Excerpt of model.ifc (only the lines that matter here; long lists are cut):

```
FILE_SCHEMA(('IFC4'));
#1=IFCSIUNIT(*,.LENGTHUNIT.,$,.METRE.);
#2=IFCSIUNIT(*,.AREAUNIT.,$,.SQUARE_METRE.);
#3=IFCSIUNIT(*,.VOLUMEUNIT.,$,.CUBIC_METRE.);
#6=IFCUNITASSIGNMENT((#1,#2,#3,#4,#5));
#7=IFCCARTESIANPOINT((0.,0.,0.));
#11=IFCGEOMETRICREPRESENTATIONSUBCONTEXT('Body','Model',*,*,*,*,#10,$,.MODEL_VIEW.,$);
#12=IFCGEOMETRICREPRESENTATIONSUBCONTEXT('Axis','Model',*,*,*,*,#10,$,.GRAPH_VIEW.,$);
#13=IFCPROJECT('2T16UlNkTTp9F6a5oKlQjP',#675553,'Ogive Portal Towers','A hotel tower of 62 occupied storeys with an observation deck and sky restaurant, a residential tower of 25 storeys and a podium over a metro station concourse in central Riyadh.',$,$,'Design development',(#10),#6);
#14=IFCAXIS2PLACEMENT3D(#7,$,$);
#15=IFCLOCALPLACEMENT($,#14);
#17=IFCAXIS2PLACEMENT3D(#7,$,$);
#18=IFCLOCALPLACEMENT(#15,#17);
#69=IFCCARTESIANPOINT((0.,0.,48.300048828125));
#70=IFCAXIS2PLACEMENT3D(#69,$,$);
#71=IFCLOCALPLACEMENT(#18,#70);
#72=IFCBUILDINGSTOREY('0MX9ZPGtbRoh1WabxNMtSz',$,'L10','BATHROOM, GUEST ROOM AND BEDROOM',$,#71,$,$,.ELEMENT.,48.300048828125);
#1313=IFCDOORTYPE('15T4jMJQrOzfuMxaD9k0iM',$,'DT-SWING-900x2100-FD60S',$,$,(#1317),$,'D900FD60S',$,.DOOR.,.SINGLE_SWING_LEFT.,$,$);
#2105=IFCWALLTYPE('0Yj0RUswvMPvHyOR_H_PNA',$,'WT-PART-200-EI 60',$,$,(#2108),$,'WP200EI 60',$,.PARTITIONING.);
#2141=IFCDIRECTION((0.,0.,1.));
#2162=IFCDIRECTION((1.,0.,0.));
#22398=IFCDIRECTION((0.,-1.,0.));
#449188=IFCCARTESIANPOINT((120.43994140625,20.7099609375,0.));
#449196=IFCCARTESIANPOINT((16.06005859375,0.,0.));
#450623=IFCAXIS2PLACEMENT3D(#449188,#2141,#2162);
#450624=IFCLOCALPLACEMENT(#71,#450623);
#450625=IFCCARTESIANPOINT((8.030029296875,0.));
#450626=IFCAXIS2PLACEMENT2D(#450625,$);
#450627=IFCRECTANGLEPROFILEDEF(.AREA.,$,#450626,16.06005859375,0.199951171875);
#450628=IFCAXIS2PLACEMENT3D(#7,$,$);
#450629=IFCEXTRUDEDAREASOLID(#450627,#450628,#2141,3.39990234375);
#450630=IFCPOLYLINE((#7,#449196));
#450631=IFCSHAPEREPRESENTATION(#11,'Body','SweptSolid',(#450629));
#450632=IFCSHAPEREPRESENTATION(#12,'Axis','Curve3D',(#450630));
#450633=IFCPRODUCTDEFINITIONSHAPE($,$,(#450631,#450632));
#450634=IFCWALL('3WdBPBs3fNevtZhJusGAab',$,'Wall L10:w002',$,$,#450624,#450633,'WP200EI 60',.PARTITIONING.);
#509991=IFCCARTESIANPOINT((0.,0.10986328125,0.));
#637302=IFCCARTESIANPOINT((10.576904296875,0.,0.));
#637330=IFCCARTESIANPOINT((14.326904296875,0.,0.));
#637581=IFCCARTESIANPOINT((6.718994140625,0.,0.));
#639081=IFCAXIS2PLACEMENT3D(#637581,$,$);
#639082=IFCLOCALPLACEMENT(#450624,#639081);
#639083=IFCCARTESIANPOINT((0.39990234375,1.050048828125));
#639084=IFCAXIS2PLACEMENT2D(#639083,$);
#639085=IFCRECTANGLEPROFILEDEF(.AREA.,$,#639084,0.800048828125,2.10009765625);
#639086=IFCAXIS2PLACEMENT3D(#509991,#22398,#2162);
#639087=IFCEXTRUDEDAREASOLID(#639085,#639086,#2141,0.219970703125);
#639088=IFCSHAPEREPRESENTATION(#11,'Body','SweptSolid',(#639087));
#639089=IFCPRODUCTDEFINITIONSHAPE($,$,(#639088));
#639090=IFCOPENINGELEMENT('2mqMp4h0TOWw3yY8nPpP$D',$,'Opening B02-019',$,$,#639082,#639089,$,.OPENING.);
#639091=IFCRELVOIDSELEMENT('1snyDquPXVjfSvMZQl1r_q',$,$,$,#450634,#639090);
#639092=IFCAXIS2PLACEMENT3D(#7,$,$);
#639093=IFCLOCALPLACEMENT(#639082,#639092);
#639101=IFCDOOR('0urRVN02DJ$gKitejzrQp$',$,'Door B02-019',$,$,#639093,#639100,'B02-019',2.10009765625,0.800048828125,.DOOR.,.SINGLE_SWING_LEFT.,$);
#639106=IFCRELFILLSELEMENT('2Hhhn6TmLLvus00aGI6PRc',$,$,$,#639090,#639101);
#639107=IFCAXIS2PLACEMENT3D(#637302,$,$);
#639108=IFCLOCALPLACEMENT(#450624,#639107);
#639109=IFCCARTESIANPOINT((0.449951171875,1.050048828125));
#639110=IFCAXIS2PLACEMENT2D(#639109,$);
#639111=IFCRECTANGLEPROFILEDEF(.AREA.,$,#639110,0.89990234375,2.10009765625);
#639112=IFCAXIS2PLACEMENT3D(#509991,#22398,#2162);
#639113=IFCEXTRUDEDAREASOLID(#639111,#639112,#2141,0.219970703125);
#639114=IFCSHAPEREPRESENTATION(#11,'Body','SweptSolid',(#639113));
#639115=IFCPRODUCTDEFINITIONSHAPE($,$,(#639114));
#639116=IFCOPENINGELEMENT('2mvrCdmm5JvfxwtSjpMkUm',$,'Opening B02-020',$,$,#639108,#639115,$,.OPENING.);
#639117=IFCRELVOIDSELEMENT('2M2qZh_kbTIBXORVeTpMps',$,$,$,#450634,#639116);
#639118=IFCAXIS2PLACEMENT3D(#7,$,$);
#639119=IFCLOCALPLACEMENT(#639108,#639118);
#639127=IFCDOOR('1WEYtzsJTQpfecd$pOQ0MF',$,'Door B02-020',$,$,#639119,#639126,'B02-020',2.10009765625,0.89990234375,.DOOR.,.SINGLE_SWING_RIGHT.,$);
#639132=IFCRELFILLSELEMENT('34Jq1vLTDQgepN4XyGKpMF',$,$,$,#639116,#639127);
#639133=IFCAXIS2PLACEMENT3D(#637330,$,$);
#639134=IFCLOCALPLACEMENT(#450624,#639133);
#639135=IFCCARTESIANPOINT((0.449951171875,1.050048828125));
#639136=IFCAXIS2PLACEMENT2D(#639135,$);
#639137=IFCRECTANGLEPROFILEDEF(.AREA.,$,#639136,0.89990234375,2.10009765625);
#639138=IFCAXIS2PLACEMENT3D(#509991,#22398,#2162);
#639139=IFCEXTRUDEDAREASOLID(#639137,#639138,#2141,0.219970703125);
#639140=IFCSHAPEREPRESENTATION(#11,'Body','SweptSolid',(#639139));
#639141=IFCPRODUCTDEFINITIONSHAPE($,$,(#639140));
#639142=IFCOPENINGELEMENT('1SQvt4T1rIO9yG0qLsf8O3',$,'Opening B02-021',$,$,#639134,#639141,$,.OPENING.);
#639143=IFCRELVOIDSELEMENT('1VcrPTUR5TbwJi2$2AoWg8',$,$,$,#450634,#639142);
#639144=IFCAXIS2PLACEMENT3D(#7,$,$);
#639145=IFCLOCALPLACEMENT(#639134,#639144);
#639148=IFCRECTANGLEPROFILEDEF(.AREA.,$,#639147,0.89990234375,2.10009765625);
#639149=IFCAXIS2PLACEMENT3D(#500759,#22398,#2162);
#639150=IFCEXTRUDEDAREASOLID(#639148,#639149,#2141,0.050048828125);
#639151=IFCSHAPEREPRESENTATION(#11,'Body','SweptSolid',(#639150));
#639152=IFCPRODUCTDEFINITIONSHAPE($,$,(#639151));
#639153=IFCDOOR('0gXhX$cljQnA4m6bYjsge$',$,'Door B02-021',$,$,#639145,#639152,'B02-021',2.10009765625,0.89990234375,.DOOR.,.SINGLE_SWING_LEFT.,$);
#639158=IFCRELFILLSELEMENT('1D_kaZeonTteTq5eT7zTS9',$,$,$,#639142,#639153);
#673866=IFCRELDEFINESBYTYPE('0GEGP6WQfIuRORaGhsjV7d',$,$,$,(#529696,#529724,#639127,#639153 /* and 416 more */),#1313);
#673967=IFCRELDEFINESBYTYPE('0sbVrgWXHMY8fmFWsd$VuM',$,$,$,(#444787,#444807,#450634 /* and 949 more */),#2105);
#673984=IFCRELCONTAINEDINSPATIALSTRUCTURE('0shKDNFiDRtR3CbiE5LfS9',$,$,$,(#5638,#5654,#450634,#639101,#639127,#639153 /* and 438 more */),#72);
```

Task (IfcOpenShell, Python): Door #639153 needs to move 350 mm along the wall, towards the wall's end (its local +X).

```python
import ifcopenshell
import ifcopenshell.api.geometry
import ifcopenshell.util.placement
import ifcopenshell.util.unit

model = ifcopenshell.open("model.ifc")
unit_scale = ifcopenshell.util.unit.calculate_unit_scale(model)

door = model.by_guid("0gXhX$cljQnA4m6bYjsge$")
opening = door.FillsVoids[0].RelatingOpeningElement
wall = opening.VoidsElements[0].RelatingBuildingElement

wall_matrix = ifcopenshell.util.placement.get_local_placement(wall.ObjectPlacement)
shift = wall_matrix[:3, 0] * 0.35 / unit_scale
before = ifcopenshell.util.placement.get_local_placement(door.ObjectPlacement)[:3, 3].copy()

# The door is placed relative to its opening, so it follows when the opening moves.
matrix = ifcopenshell.util.placement.get_local_placement(opening.ObjectPlacement)
matrix[:3, 3] += shift
ifcopenshell.api.geometry.edit_object_placement(
    model, product=opening, matrix=matrix, is_si=False, should_transform_children=True
)

after = ifcopenshell.util.placement.get_local_placement(door.ObjectPlacement)[:3, 3]
print("door moved by", (after - before).round(3) + 0.0)

model.write("model_rev.ifc")
```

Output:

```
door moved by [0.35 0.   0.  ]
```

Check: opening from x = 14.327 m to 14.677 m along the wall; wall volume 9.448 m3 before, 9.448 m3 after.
